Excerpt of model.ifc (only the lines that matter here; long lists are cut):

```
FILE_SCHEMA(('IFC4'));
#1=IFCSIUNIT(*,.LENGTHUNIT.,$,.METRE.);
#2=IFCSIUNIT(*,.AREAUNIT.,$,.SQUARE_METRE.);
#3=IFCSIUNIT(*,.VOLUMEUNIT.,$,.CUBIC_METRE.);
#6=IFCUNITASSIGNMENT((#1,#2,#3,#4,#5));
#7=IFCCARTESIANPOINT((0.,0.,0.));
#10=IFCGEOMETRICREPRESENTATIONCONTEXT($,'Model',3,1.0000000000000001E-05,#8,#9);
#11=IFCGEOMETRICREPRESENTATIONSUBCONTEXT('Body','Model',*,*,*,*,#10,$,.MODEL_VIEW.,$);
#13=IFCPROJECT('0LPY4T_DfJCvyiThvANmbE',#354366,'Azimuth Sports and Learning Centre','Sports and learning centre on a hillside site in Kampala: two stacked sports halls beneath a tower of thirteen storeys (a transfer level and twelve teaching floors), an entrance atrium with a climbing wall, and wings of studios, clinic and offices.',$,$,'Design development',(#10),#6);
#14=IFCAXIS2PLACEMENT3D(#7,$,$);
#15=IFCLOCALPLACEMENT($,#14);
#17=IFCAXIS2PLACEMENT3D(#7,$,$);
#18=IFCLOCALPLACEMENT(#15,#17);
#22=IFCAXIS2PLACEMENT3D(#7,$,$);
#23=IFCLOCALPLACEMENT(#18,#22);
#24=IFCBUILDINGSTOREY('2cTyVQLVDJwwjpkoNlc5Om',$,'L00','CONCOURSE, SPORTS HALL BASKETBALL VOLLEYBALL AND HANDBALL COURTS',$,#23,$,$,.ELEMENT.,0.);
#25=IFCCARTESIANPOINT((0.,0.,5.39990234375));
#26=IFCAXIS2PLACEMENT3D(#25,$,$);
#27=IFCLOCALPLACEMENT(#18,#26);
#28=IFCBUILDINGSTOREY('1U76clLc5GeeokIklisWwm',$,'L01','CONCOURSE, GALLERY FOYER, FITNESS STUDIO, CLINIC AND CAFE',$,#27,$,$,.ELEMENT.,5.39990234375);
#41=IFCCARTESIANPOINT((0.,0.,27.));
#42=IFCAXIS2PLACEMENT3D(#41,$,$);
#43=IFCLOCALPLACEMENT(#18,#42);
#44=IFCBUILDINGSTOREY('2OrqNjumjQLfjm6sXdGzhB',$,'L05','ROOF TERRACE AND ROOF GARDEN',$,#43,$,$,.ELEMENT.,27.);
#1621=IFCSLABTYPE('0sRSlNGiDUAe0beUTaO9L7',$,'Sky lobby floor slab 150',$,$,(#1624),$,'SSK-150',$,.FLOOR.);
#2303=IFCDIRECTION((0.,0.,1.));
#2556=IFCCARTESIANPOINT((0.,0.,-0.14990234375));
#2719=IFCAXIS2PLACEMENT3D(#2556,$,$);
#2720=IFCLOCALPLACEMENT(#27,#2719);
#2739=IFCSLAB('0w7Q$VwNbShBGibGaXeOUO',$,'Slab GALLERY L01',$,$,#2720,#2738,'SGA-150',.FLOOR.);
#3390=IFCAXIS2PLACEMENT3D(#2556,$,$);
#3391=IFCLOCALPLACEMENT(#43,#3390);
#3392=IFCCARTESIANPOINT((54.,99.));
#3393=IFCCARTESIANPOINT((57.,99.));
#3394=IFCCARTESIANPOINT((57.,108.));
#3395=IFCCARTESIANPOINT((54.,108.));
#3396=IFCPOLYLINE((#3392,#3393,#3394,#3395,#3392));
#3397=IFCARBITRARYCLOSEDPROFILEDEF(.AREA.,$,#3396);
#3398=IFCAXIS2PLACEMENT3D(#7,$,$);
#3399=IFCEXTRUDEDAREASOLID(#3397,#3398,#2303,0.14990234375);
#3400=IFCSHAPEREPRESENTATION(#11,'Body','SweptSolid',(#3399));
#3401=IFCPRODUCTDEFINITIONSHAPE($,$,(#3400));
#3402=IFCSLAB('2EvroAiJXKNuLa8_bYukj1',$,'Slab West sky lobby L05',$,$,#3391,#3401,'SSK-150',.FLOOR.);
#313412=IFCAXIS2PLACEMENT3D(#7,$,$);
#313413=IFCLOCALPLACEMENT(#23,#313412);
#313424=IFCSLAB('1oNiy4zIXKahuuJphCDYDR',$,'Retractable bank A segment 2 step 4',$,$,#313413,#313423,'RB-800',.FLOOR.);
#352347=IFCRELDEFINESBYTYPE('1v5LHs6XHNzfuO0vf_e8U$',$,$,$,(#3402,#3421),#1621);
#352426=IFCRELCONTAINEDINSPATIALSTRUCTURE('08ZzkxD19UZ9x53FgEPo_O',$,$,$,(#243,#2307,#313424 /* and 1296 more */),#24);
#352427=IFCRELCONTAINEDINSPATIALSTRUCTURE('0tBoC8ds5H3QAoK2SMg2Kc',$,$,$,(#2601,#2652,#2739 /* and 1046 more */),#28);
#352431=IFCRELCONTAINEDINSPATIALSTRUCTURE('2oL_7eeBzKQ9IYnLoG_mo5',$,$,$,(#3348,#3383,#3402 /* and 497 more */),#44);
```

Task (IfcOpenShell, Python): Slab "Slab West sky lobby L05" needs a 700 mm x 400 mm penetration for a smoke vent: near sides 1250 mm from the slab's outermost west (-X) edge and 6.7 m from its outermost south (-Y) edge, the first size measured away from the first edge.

```python
import numpy as np
import ifcopenshell
import ifcopenshell.api.feature
import ifcopenshell.api.geometry
import ifcopenshell.api.root
import ifcopenshell.geom
import ifcopenshell.util.placement
import ifcopenshell.util.representation
import ifcopenshell.util.shape
import ifcopenshell.util.unit

model = ifcopenshell.open("model.ifc")
unit_scale = ifcopenshell.util.unit.calculate_unit_scale(model)
settings = ifcopenshell.geom.settings()


def volume(element):
    """Net volume in cubic metres, openings subtracted."""
    shape = ifcopenshell.geom.create_shape(settings, element)
    return ifcopenshell.util.shape.get_volume(shape.geometry)


slab = model.by_guid("2EvroAiJXKNuLa8_bYukj1")
before = volume(slab)

# Extent in the slab's own axes, in metres. The edges named are its -X and -Y sides.
slab_shape = ifcopenshell.geom.create_shape(settings, slab)
vertices = ifcopenshell.util.shape.get_vertices(slab_shape.geometry)
x_min, y_min, bottom = vertices.min(axis=0)
top = vertices[:, 2].max()

opening = ifcopenshell.api.root.create_entity(model, ifc_class="IfcOpeningElement", name="Smoke vent opening", predefined_type="OPENING")
context = ifcopenshell.util.representation.get_context(model, "Model", "Body", "MODEL_VIEW")
width, depth = 0.7, 0.4
outline = [(0.0, 0.0), (width, 0.0), (width, depth), (0.0, depth), (0.0, 0.0)]
# Overshoot both faces by 50 mm so the cut is clean.
shape = ifcopenshell.api.geometry.add_slab_representation(
    model, context=context, depth=top - bottom + 0.1, polyline=outline
)
ifcopenshell.api.geometry.assign_representation(model, product=opening, representation=shape)

matrix = ifcopenshell.util.placement.get_local_placement(slab.ObjectPlacement)
matrix[:, 3] = matrix @ np.append(np.array([x_min + 1.25, y_min + 6.7, bottom - 0.05]) / unit_scale, 1.0)
ifcopenshell.api.geometry.edit_object_placement(model, product=opening, matrix=matrix, is_si=False)
ifcopenshell.api.feature.add_feature(model, feature=opening, element=slab)

after = volume(slab)

print(f"slab volume {before:.3f} -> {after:.3f} m3")

model.write("model_rev.ifc")
```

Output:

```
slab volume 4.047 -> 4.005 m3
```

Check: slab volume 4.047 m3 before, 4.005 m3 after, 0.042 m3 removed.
